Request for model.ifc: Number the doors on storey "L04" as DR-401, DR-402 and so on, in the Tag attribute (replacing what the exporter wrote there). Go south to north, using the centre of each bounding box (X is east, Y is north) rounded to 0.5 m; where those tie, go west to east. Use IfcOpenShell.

First a look at what the model holds.

```python
import ifcopenshell
import ifcopenshell.util.element
import ifcopenshell.util.placement

model = ifcopenshell.open("model.ifc")
print(model.schema)
storey = next(s for s in model.by_type("IfcBuildingStorey") if s.Name == "L04")
doors = [e for e in ifcopenshell.util.element.get_decomposition(storey) if e.is_a("IfcDoor")]
for e in sorted(doors, key=lambda e: e.id()):
    origin = ifcopenshell.util.placement.get_local_placement(e.ObjectPlacement)[:3, 3]
    print(e.id(), e.Tag, e.Name, origin.round(2) + 0.0, sep=" | ")
```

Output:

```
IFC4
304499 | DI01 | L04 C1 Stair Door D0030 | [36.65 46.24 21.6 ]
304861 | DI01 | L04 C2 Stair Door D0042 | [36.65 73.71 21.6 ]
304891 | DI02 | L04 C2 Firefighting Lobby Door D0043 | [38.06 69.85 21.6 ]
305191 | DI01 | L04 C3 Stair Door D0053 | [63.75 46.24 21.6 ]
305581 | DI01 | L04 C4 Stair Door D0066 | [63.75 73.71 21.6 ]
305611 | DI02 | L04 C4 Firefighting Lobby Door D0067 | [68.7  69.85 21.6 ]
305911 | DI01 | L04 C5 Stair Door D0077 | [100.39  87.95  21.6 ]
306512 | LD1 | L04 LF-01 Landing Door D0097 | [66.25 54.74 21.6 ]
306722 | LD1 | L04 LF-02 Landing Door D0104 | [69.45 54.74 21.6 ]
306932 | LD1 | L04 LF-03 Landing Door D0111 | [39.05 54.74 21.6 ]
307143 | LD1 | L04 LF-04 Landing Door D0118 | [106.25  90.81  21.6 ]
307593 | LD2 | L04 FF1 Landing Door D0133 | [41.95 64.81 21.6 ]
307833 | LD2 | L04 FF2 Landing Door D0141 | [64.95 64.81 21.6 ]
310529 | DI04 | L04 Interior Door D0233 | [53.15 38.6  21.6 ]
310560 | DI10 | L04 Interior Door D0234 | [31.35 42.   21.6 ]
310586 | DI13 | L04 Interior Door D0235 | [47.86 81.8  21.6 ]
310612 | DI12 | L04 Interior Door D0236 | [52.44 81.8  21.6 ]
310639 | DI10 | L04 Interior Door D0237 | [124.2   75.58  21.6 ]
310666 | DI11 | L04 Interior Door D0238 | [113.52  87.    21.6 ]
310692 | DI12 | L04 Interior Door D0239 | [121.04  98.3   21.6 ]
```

```python
import ifcopenshell
import ifcopenshell.geom
import ifcopenshell.util.element
import ifcopenshell.util.shape

model = ifcopenshell.open("model.ifc")
settings = ifcopenshell.geom.settings()
settings.set("use-world-coords", True)


def centre(element):
    shape = ifcopenshell.geom.create_shape(settings, element)
    return ifcopenshell.util.shape.get_bbox_centroid(shape.geometry)


storey = next(s for s in model.by_type("IfcBuildingStorey") if s.Name == "L04")
doors = [e for e in ifcopenshell.util.element.get_decomposition(storey) if e.is_a("IfcDoor")]

# Insertion points can sit at a corner or the storey origin, so sort by the geometry (in metres).
centres = {e: centre(e) for e in doors}
doors.sort(key=lambda e: (round(centres[e][1] / 0.5), centres[e][0]))

for i, e in enumerate(doors, start=1):
    number = f"DR-4{i:02d}"
    e.Tag = number
    print(e.id(), number)

model.write("model_updated.ifc")
```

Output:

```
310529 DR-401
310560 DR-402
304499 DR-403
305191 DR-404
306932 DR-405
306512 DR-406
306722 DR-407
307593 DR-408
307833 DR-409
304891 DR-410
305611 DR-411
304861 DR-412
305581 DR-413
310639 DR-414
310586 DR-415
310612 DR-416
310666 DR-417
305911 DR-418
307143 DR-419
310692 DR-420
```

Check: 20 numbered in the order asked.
